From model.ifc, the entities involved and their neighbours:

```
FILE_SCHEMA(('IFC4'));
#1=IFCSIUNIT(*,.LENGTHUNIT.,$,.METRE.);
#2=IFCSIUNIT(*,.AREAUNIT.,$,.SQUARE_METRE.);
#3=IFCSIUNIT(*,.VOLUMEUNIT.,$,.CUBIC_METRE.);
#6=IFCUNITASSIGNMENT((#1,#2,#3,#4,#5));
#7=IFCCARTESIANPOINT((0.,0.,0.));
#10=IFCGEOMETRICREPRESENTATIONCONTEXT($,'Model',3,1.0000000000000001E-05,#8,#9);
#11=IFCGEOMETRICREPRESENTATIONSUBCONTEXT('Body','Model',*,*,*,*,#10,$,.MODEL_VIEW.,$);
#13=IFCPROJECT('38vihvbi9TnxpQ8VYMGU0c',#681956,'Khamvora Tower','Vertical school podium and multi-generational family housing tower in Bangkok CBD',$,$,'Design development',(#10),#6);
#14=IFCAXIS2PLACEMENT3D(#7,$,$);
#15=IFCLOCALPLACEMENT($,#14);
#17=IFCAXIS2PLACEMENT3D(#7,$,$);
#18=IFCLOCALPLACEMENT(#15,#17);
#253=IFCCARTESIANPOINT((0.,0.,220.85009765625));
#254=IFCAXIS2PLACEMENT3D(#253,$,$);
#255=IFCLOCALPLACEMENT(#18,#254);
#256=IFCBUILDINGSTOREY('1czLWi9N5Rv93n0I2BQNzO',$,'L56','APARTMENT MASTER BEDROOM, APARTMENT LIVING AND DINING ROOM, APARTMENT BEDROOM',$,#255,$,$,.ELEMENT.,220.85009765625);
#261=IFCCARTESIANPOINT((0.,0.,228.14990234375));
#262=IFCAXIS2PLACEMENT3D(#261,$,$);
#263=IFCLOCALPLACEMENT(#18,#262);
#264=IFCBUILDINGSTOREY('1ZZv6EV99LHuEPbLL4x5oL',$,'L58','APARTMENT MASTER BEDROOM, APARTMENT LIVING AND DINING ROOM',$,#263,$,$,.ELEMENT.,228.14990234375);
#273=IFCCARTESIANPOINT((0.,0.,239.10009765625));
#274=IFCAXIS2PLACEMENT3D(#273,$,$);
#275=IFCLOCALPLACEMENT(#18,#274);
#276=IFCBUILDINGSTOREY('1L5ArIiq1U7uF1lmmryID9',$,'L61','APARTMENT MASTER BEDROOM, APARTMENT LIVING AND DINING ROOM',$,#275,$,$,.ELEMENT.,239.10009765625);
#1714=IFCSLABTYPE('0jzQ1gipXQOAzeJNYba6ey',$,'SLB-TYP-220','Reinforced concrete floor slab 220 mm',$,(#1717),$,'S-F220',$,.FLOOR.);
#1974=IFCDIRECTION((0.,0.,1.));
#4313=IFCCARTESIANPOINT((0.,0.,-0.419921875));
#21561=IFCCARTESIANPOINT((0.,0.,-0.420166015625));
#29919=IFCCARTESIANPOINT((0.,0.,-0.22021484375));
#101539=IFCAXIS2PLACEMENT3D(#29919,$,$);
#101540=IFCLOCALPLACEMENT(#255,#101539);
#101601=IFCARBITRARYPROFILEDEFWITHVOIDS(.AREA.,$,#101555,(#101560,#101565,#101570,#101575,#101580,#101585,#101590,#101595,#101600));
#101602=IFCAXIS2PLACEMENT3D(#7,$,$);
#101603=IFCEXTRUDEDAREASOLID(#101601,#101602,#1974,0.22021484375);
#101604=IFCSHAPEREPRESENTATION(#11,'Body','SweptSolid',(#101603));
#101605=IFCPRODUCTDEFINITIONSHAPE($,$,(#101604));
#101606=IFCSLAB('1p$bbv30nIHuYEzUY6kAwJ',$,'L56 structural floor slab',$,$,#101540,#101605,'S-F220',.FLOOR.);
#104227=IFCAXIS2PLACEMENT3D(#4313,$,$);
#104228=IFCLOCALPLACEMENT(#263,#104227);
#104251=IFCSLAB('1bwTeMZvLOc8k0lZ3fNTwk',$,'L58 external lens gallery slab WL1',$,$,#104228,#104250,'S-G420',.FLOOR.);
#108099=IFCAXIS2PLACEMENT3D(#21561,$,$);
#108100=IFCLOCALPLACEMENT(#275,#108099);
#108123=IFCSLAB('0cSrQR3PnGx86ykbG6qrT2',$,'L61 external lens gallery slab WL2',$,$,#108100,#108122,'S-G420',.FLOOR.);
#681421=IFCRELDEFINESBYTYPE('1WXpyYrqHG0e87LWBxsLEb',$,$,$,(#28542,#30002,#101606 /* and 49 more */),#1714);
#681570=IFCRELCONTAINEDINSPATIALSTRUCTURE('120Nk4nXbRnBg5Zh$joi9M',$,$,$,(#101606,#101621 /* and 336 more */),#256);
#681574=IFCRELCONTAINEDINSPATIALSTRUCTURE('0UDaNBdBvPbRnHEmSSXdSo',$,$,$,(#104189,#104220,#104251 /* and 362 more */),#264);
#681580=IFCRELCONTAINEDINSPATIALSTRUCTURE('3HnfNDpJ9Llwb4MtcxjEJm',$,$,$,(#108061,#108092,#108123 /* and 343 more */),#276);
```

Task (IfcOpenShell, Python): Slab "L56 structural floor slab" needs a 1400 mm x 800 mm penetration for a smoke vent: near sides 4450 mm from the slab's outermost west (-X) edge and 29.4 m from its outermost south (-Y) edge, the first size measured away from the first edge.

```python
import numpy as np
import ifcopenshell
import ifcopenshell.api.feature
import ifcopenshell.api.geometry
import ifcopenshell.api.root
import ifcopenshell.geom
import ifcopenshell.util.placement
import ifcopenshell.util.representation
import ifcopenshell.util.shape
import ifcopenshell.util.unit

model = ifcopenshell.open("model.ifc")
unit_scale = ifcopenshell.util.unit.calculate_unit_scale(model)
settings = ifcopenshell.geom.settings()


def volume(element):
    """Net volume in cubic metres, openings subtracted."""
    shape = ifcopenshell.geom.create_shape(settings, element)
    return ifcopenshell.util.shape.get_volume(shape.geometry)


slab = model.by_guid("1p$bbv30nIHuYEzUY6kAwJ")
before = volume(slab)

# Extent in the slab's own axes, in metres. The edges named are its -X and -Y sides.
slab_shape = ifcopenshell.geom.create_shape(settings, slab)
vertices = ifcopenshell.util.shape.get_vertices(slab_shape.geometry)
x_min, y_min, bottom = vertices.min(axis=0)
top = vertices[:, 2].max()

opening = ifcopenshell.api.root.create_entity(model, ifc_class="IfcOpeningElement", name="Smoke vent opening", predefined_type="OPENING")
context = ifcopenshell.util.representation.get_context(model, "Model", "Body", "MODEL_VIEW")
width, depth = 1.4, 0.8
outline = [(0.0, 0.0), (width, 0.0), (width, depth), (0.0, depth), (0.0, 0.0)]
# Overshoot both faces by 50 mm so the cut is clean.
shape = ifcopenshell.api.geometry.add_slab_representation(
    model, context=context, depth=top - bottom + 0.1, polyline=outline
)
ifcopenshell.api.geometry.assign_representation(model, product=opening, representation=shape)

matrix = ifcopenshell.util.placement.get_local_placement(slab.ObjectPlacement)
matrix[:, 3] = matrix @ np.append(np.array([x_min + 4.45, y_min + 29.4, bottom - 0.05]) / unit_scale, 1.0)
ifcopenshell.api.geometry.edit_object_placement(model, product=opening, matrix=matrix, is_si=False)
ifcopenshell.api.feature.add_feature(model, feature=opening, element=slab)

after = volume(slab)

print(f"slab volume {before:.3f} -> {after:.3f} m3")

model.write("model_edited.ifc")
```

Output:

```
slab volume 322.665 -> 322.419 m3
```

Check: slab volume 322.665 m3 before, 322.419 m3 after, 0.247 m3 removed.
